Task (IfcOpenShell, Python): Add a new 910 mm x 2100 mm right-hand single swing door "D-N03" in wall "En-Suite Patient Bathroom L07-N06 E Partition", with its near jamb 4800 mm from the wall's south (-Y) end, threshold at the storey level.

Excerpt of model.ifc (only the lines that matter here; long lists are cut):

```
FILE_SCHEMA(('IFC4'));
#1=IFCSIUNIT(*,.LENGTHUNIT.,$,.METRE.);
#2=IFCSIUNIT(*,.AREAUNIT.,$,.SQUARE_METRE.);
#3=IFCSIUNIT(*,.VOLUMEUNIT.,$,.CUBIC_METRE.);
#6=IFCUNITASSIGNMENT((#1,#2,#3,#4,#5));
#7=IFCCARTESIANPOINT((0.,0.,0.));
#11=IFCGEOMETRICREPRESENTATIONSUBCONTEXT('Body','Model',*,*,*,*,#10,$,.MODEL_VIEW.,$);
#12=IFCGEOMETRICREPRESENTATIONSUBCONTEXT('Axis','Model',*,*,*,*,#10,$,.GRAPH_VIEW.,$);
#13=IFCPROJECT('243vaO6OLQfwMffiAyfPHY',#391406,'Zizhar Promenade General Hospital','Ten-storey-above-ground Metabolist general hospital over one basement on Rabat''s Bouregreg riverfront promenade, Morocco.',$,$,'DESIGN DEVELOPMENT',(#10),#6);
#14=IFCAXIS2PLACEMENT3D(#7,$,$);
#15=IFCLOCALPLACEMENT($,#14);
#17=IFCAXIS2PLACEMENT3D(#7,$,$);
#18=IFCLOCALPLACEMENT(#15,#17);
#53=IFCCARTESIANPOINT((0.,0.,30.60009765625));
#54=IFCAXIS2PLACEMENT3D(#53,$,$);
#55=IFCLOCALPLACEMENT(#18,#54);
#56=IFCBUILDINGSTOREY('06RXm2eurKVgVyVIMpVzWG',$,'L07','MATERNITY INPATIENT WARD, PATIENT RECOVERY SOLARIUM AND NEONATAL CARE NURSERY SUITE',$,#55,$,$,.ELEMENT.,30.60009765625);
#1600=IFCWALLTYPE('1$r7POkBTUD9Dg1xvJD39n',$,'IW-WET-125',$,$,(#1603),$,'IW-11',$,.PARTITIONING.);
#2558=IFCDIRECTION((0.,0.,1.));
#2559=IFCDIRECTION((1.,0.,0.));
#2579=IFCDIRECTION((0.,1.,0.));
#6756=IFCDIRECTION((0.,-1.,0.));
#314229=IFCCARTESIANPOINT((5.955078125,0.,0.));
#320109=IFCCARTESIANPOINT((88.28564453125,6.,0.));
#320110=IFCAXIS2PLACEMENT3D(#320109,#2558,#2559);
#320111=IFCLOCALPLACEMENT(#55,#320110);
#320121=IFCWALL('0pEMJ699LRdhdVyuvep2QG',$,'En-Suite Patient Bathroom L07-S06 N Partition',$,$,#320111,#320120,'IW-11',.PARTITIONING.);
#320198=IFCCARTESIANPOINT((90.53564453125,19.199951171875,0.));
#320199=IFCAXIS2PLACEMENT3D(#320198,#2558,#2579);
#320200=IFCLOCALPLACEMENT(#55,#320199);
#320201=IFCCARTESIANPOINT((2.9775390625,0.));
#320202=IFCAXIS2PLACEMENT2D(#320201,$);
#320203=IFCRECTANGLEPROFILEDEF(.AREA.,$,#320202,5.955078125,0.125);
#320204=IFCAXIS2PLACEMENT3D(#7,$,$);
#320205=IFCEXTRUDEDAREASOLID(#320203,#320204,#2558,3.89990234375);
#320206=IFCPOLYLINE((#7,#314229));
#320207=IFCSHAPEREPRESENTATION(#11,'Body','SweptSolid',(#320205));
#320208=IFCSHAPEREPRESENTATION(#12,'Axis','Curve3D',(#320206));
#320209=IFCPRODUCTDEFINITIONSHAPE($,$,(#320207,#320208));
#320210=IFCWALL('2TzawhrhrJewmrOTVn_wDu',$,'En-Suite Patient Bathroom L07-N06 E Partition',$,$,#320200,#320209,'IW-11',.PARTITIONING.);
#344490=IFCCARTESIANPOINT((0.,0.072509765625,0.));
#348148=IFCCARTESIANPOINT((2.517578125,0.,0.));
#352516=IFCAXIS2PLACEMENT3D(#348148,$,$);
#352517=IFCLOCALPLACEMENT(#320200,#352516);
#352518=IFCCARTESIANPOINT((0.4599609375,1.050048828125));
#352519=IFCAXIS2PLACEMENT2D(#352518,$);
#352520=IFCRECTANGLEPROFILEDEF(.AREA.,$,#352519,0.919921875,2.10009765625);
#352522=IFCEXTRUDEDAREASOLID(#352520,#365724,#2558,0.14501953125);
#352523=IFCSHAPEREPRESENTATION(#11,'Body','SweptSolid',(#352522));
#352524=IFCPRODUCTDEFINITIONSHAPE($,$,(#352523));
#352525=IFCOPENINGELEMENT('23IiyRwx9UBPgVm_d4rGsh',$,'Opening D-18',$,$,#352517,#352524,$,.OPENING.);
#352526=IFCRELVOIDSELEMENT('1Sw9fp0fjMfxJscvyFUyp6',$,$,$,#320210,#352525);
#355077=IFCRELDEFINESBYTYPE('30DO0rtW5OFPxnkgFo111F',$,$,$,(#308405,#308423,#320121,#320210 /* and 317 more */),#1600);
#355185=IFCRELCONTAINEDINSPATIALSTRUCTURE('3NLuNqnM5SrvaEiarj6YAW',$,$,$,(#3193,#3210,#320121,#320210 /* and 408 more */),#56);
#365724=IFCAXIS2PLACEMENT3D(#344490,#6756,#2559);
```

```python
import numpy as np
import ifcopenshell
import ifcopenshell.api.feature
import ifcopenshell.api.geometry
import ifcopenshell.api.root
import ifcopenshell.api.spatial
import ifcopenshell.geom
import ifcopenshell.util.element
import ifcopenshell.util.placement
import ifcopenshell.util.representation
import ifcopenshell.util.shape
import ifcopenshell.util.unit

model = ifcopenshell.open("model.ifc")
unit_scale = ifcopenshell.util.unit.calculate_unit_scale(model)
settings = ifcopenshell.geom.settings()


def volume(element):
    """Net volume in cubic metres, openings subtracted."""
    shape = ifcopenshell.geom.create_shape(settings, element)
    return ifcopenshell.util.shape.get_volume(shape.geometry)


wall = model.by_guid("2TzawhrhrJewmrOTVn_wDu")
storey = ifcopenshell.util.element.get_container(wall, ifc_class="IfcBuildingStorey")
context = ifcopenshell.util.representation.get_context(model, "Model", "Body", "MODEL_VIEW")
before = volume(wall)

width, height, from_end, sill = 0.91, 2.1, 4.8, 0.0  # metres

# The wall runs along its own X axis, and the end named is its -X end.
wall_shape = ifcopenshell.geom.create_shape(settings, wall)
x, y, z = ifcopenshell.util.shape.get_vertices(wall_shape.geometry).T
start = x.min() + from_end
face, thickness = float(y.min()), float(y.max() - y.min())
wall_matrix = ifcopenshell.util.placement.get_local_placement(wall.ObjectPlacement)
level = ifcopenshell.util.placement.get_local_placement(storey.ObjectPlacement)[2, 3]


def in_wall(x, y):
    """Placement at x, y metres in the wall's axes, at sill height."""
    matrix = wall_matrix.copy()
    matrix[:, 3] = wall_matrix @ np.array([x / unit_scale, y / unit_scale, 0.0, 1.0])
    matrix[2, 3] = level + sill / unit_scale
    return matrix


# Opening: a box that overshoots both wall faces by 50 mm.
opening = ifcopenshell.api.root.create_entity(model, ifc_class="IfcOpeningElement", predefined_type="OPENING")
box = ifcopenshell.api.geometry.add_wall_representation(
    model, context=context, length=width, height=height, thickness=thickness + 0.1
)
ifcopenshell.api.geometry.assign_representation(model, product=opening, representation=box)
ifcopenshell.api.geometry.edit_object_placement(model, product=opening, matrix=in_wall(start, face - 0.05), is_si=False)
ifcopenshell.api.feature.add_feature(model, feature=opening, element=wall)

door = ifcopenshell.api.root.create_entity(model, ifc_class="IfcDoor", name="D-N03", predefined_type="DOOR")
door.OverallWidth, door.OverallHeight = width / unit_scale, height / unit_scale
door.OperationType = "SINGLE_SWING_RIGHT"
body = ifcopenshell.api.geometry.add_door_representation(
    model,
    context=context,
    overall_width=door.OverallWidth,
    overall_height=door.OverallHeight,
    operation_type="SINGLE_SWING_RIGHT",
    lining_properties={"LiningDepth": thickness / unit_scale, "ThresholdDepth": thickness / unit_scale},
)
ifcopenshell.api.geometry.assign_representation(model, product=door, representation=body)
ifcopenshell.api.spatial.assign_container(model, products=[door], relating_structure=storey)
ifcopenshell.api.feature.add_filling(model, opening=opening, element=door)

# The lining spans the wall, so the door starts at the wall face.
ifcopenshell.api.geometry.edit_object_placement(model, product=door, matrix=in_wall(start, face), is_si=False)

after = volume(wall)

print(f"wall volume {before:.3f} -> {after:.3f} m3")

model.write("model_v2.ifc")
```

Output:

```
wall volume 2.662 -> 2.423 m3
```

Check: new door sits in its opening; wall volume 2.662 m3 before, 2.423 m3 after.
